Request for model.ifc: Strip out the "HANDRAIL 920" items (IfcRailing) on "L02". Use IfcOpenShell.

First a look at what the model holds.

```python
import ifcopenshell
import ifcopenshell.util.element

model = ifcopenshell.open("model.ifc")
print(model.schema)
storey = next(s for s in model.by_type("IfcBuildingStorey") if s.Name == "L02")
railings = [e for e in ifcopenshell.util.element.get_decomposition(storey) if e.is_a("IfcRailing")]
seen = {}
for e in railings:
    element_type = ifcopenshell.util.element.get_type(e)
    name = element_type.Name if element_type not in (None, e) else None
    seen[name] = seen.get(name, 0) + 1
for name, count in sorted(seen.items(), key=str):
    print(count, "x", name)
```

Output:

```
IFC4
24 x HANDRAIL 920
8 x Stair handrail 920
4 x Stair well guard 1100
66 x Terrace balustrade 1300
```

```python
import ifcopenshell
import ifcopenshell.api.root
import ifcopenshell.util.element

model = ifcopenshell.open("model.ifc")

storey = next(s for s in model.by_type("IfcBuildingStorey") if s.Name == "L02")
railings = [e for e in ifcopenshell.util.element.get_decomposition(storey) if e.is_a("IfcRailing")]
targets = [e for e in railings if (t := ifcopenshell.util.element.get_type(e)) not in (None, e) and t.Name == "HANDRAIL 920"]

for e in targets:
    ifcopenshell.api.root.remove_product(model, product=e)
print(len(targets), "removed")

model.write("model_updated.ifc")
```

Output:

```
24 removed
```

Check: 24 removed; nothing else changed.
